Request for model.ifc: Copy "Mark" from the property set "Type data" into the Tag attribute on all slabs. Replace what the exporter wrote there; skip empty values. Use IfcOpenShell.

First a look at what the model holds.

```python
import ifcopenshell
import ifcopenshell.util.element

model = ifcopenshell.open("model.ifc")
print(model.schema)
slabs = model.by_type("IfcSlab")
print(len(slabs), "slabs")
for e in slabs[:8]:
    source = ifcopenshell.util.element.get_pset(e, "Type data", "Mark")
    target = e.Tag
    print(e.id(), repr(source), repr(target), sep=" | ")
```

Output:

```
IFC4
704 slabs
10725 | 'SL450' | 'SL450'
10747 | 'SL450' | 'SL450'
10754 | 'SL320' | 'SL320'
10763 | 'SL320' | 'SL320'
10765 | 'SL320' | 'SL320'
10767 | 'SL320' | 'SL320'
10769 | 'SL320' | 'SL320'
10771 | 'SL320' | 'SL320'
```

```python
import ifcopenshell
import ifcopenshell.util.element

model = ifcopenshell.open("model.ifc")

count = 0
for e in model.by_type("IfcSlab"):
    value = ifcopenshell.util.element.get_pset(e, "Type data", "Mark")
    current = e.Tag
    if not value or not value.strip() or current == value:
        continue
    e.Tag = value
    count += 1

print(count, "slabs updated")

model.write("model-out.ifc")
```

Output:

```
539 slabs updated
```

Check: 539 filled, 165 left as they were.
